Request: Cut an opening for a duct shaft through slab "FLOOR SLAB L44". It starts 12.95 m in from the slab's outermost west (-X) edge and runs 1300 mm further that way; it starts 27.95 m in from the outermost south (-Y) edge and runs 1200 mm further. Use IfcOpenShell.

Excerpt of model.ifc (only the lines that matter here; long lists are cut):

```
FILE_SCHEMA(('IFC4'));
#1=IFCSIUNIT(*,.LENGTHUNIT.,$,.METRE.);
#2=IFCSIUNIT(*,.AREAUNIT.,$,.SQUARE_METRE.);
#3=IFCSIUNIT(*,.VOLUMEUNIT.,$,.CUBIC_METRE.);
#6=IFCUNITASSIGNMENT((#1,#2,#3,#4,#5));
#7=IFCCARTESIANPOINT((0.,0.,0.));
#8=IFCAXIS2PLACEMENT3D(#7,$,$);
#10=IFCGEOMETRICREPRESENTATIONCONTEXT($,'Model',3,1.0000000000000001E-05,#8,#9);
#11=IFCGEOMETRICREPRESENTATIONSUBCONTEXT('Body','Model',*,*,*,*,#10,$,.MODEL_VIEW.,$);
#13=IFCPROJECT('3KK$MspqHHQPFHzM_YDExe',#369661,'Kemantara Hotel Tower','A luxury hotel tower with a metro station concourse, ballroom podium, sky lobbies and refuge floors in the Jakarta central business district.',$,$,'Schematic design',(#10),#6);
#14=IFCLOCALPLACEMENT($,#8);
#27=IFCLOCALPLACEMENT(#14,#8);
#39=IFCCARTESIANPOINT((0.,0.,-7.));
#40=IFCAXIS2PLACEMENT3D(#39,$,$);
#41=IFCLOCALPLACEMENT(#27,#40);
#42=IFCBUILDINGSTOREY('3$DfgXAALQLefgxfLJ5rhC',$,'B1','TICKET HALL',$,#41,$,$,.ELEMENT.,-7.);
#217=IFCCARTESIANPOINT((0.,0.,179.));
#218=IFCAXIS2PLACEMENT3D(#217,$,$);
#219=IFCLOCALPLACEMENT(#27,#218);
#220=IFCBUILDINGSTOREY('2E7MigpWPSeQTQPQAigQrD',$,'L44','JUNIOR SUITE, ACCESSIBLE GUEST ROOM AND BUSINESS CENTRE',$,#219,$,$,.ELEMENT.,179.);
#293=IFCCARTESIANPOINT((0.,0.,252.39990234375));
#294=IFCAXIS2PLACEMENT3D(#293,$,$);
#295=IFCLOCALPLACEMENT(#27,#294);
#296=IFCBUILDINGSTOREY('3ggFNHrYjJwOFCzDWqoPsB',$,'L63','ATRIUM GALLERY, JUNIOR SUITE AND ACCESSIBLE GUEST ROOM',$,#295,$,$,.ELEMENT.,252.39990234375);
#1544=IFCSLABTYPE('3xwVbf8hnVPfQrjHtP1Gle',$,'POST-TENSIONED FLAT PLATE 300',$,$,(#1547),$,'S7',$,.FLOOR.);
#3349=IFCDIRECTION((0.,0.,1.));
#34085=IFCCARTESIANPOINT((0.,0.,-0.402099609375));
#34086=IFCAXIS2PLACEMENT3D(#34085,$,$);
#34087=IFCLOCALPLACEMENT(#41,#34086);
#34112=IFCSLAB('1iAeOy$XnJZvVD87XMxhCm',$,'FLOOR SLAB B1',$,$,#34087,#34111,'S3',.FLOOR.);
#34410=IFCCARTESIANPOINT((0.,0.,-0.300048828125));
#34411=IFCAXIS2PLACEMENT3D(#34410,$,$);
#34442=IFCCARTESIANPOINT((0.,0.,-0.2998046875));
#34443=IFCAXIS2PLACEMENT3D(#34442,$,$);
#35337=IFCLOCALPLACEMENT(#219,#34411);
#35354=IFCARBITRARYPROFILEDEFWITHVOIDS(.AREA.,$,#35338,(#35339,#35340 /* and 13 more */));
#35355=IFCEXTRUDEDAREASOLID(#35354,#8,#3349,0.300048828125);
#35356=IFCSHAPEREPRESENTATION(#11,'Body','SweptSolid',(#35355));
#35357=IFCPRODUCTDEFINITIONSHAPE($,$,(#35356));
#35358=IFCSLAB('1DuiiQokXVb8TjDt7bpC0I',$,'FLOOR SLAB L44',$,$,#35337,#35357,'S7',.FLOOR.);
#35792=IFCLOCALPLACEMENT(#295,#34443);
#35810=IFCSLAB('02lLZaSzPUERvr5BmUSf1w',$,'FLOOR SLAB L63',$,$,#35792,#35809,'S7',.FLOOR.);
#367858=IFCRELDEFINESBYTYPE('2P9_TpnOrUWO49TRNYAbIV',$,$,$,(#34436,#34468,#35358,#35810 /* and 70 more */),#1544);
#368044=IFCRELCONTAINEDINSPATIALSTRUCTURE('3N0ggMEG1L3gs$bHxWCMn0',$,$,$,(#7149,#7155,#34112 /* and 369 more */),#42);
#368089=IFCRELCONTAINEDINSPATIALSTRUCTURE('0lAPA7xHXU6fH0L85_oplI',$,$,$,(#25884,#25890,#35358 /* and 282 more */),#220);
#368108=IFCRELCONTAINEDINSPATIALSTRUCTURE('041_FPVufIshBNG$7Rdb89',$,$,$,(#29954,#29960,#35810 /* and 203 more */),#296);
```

```python
import numpy as np
import ifcopenshell
import ifcopenshell.api.feature
import ifcopenshell.api.geometry
import ifcopenshell.api.root
import ifcopenshell.geom
import ifcopenshell.util.placement
import ifcopenshell.util.representation
import ifcopenshell.util.shape
import ifcopenshell.util.unit

model = ifcopenshell.open("model.ifc")
unit_scale = ifcopenshell.util.unit.calculate_unit_scale(model)
settings = ifcopenshell.geom.settings()


def volume(element):
    """Net volume in cubic metres, openings subtracted."""
    shape = ifcopenshell.geom.create_shape(settings, element)
    return ifcopenshell.util.shape.get_volume(shape.geometry)


slab = model.by_id(35358)
before = volume(slab)

# Extent in the slab's own axes, in metres. The edges named are its -X and -Y sides.
slab_shape = ifcopenshell.geom.create_shape(settings, slab)
vertices = ifcopenshell.util.shape.get_vertices(slab_shape.geometry)
x_min, y_min, bottom = vertices.min(axis=0)
top = vertices[:, 2].max()

opening = ifcopenshell.api.root.create_entity(model, ifc_class="IfcOpeningElement", name="Duct shaft opening", predefined_type="OPENING")
context = ifcopenshell.util.representation.get_context(model, "Model", "Body", "MODEL_VIEW")
width, depth = 1.3, 1.2
outline = [(0.0, 0.0), (width, 0.0), (width, depth), (0.0, depth), (0.0, 0.0)]
# Overshoot both faces by 50 mm so the cut is clean.
shape = ifcopenshell.api.geometry.add_slab_representation(
    model, context=context, depth=top - bottom + 0.1, polyline=outline
)
ifcopenshell.api.geometry.assign_representation(model, product=opening, representation=shape)

matrix = ifcopenshell.util.placement.get_local_placement(slab.ObjectPlacement)
matrix[:, 3] = matrix @ np.append(np.array([x_min + 12.95, y_min + 27.95, bottom - 0.05]) / unit_scale, 1.0)
ifcopenshell.api.geometry.edit_object_placement(model, product=opening, matrix=matrix, is_si=False)
ifcopenshell.api.feature.add_feature(model, feature=opening, element=slab)

after = volume(slab)

print(f"slab volume {before:.3f} -> {after:.3f} m3")

model.write("model_v2.ifc")
```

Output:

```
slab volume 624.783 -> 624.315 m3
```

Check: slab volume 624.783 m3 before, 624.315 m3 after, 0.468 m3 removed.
